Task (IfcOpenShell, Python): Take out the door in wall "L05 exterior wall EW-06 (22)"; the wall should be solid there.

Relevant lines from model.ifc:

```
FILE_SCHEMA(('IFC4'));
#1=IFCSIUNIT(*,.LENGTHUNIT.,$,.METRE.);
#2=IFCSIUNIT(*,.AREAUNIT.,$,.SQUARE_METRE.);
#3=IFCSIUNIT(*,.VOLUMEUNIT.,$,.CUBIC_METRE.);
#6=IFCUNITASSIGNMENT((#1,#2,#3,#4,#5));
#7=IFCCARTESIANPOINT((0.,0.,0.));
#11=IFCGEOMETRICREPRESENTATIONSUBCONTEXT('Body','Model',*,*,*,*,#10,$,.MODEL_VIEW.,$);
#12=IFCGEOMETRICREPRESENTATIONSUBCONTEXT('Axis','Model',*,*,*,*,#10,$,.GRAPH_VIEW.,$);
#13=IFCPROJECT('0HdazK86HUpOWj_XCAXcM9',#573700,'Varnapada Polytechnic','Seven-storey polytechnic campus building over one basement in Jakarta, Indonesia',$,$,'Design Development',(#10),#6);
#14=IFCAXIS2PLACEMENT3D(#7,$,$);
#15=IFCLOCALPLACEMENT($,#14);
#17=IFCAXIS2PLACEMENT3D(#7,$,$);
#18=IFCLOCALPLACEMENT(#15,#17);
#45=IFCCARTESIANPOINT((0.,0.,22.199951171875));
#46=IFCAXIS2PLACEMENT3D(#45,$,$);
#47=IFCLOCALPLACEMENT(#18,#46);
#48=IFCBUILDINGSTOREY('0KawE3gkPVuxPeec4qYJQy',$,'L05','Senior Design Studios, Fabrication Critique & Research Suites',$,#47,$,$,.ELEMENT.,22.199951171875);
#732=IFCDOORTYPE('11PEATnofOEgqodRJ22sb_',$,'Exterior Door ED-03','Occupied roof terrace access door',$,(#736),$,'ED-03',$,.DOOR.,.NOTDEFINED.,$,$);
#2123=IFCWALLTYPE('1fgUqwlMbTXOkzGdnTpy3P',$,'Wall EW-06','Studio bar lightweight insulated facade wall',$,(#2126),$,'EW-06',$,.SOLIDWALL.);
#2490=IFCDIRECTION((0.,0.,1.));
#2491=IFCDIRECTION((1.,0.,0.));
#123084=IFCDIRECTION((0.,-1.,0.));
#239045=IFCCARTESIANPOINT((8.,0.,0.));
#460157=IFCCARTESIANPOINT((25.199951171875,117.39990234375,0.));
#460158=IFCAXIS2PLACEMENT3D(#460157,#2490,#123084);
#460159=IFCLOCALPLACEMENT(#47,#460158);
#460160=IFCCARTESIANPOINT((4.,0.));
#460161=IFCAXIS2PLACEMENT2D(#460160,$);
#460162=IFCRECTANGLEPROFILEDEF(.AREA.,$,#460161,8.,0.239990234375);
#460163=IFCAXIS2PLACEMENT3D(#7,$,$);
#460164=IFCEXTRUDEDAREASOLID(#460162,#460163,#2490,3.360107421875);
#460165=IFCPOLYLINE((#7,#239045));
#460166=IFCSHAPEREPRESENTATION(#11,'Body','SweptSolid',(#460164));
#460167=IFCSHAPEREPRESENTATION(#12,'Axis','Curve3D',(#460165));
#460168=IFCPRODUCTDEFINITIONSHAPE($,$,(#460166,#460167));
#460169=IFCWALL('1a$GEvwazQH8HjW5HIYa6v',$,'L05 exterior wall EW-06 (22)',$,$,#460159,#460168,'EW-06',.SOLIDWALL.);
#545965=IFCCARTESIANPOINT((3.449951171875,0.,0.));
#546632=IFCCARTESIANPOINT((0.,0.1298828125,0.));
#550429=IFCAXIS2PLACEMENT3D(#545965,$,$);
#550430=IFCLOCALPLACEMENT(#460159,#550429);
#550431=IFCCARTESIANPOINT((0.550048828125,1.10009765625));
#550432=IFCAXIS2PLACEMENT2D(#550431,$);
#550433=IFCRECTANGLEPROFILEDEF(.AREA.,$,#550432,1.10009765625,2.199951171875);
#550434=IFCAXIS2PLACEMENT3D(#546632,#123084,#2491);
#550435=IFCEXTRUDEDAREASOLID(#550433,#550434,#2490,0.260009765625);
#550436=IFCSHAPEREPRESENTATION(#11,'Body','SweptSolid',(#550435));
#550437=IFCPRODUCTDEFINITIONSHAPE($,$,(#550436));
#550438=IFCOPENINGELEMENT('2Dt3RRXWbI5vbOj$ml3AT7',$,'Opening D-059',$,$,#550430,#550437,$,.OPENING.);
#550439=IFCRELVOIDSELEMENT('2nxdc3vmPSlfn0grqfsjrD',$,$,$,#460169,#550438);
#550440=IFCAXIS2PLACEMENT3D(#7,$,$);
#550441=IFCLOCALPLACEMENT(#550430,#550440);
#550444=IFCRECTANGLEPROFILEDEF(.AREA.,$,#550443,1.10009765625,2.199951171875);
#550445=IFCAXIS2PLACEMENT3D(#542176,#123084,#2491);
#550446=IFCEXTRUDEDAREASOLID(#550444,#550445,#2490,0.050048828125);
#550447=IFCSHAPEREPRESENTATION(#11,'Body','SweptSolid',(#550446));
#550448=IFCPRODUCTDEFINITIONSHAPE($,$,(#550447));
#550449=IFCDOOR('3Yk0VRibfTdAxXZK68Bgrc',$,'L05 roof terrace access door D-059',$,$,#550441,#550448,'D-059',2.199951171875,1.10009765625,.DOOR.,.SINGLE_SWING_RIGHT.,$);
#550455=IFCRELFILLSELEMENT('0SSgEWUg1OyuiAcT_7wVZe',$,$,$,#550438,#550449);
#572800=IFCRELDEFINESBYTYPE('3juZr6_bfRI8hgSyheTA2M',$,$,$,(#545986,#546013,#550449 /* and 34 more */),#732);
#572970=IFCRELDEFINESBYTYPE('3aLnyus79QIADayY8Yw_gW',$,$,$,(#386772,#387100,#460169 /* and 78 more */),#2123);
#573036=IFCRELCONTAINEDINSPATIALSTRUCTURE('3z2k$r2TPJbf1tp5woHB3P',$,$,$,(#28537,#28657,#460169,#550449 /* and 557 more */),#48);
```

```python
import ifcopenshell
import ifcopenshell.api.feature
import ifcopenshell.api.root
import ifcopenshell.geom
import ifcopenshell.util.shape

model = ifcopenshell.open("model.ifc")
settings = ifcopenshell.geom.settings()


def volume(element):
    """Net volume in cubic metres, openings subtracted."""
    shape = ifcopenshell.geom.create_shape(settings, element)
    return ifcopenshell.util.shape.get_volume(shape.geometry)


door = model.by_guid("3Yk0VRibfTdAxXZK68Bgrc")
opening = door.FillsVoids[0].RelatingOpeningElement
wall = opening.VoidsElements[0].RelatingBuildingElement
before = volume(wall)

ifcopenshell.api.root.remove_product(model, product=door)
ifcopenshell.api.feature.remove_feature(model, feature=opening)

after = volume(wall)

print(f"wall volume {before:.3f} -> {after:.3f} m3")

model.write("model-out.ifc")
```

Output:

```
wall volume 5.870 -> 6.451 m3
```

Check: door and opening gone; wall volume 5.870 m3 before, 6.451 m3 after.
